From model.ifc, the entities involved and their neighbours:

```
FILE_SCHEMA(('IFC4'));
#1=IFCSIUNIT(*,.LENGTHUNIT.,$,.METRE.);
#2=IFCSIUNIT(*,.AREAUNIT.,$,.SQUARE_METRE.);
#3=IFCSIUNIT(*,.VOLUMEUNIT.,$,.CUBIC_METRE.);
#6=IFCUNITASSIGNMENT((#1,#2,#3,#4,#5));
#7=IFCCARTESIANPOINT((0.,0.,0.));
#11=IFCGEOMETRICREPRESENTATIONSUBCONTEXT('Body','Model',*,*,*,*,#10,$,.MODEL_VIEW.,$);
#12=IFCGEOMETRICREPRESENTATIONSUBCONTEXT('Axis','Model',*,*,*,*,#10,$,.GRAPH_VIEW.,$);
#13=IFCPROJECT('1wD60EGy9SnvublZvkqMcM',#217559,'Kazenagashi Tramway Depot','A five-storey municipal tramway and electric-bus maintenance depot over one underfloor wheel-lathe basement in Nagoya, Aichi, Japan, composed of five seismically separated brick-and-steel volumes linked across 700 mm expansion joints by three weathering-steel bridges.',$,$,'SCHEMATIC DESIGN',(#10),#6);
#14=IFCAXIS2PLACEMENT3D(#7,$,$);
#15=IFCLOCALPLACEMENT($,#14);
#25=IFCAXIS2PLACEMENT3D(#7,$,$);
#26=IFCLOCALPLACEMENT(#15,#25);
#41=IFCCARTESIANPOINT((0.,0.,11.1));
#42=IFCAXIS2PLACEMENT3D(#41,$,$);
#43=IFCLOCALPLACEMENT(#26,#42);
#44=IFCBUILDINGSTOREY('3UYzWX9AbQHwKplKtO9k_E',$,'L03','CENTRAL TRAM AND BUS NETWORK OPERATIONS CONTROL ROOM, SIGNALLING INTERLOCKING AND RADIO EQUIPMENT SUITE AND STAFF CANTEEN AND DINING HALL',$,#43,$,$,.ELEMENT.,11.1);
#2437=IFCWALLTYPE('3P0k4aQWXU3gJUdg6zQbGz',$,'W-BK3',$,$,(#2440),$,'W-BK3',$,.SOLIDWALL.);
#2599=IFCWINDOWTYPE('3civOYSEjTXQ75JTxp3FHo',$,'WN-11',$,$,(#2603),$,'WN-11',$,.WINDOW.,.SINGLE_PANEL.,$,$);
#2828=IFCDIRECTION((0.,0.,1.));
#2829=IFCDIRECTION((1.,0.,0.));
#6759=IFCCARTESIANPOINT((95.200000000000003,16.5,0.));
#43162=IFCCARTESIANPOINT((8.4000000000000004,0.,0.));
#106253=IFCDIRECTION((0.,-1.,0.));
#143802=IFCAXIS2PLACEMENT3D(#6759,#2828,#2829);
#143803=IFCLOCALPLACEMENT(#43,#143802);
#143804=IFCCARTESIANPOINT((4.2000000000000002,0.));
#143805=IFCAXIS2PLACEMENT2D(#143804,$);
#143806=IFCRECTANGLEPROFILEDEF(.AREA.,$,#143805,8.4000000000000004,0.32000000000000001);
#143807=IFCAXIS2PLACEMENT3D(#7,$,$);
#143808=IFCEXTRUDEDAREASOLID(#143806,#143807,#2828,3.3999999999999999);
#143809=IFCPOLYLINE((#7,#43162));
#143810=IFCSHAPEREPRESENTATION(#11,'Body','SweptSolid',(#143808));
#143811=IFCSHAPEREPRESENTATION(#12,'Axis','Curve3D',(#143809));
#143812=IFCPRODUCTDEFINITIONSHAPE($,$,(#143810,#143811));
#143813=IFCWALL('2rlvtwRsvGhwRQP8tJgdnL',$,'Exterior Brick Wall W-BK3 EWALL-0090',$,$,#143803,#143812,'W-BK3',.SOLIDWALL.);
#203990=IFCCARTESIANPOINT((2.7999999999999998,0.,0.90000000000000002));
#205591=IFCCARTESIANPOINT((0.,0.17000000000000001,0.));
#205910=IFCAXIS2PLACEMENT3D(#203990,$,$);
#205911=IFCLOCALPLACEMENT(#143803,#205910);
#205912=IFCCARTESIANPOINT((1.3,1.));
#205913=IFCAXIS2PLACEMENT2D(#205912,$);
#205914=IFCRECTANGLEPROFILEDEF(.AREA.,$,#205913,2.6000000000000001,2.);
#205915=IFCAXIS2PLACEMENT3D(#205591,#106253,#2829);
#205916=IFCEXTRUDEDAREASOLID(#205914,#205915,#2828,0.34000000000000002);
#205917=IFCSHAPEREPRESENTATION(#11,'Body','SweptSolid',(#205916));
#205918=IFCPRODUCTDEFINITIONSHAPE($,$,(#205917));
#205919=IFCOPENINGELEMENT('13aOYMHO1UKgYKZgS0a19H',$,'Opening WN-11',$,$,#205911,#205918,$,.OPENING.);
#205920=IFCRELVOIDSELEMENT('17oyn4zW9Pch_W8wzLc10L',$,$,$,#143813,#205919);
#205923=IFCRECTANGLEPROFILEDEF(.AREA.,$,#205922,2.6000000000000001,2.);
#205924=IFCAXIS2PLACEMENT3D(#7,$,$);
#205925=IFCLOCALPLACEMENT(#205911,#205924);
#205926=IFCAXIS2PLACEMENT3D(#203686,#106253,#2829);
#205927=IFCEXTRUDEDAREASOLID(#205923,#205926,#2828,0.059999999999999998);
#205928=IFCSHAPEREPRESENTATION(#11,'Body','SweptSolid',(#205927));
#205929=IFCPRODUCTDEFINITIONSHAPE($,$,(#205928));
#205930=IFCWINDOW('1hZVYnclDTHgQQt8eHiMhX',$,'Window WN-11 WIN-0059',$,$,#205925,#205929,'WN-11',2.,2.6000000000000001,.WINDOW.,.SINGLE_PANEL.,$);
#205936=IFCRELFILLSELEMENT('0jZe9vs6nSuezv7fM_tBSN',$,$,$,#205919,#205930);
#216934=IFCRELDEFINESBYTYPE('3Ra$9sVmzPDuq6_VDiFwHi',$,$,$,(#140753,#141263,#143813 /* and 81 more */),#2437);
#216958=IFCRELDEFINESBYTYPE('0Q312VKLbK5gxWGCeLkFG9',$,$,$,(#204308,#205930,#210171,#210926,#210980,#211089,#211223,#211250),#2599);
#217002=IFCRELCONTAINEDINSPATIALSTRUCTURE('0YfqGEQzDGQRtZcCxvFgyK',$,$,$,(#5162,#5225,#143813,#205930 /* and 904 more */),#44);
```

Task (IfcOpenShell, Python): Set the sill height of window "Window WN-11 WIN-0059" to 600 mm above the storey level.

```python
import numpy as np
import ifcopenshell
import ifcopenshell.api.geometry
import ifcopenshell.geom
import ifcopenshell.util.element
import ifcopenshell.util.placement
import ifcopenshell.util.shape
import ifcopenshell.util.unit

model = ifcopenshell.open("model.ifc")
unit_scale = ifcopenshell.util.unit.calculate_unit_scale(model)

window = model.by_id(205930)
opening = window.FillsVoids[0].RelatingOpeningElement
storey = ifcopenshell.util.element.get_container(window, ifc_class="IfcBuildingStorey")
level = ifcopenshell.util.placement.get_local_placement(storey.ObjectPlacement)[2, 3]

# The opening's origin need not be at the sill, so measure its lowest point.
shape = ifcopenshell.geom.create_shape(ifcopenshell.geom.settings(), opening)
bottom = ifcopenshell.util.shape.get_shape_bottom_elevation(shape, shape.geometry) / unit_scale
dz = level + 0.6 - bottom

shift = np.array([0.0, 0.0, dz])
# The window is placed relative to its opening, so it follows when the opening moves.
matrix = ifcopenshell.util.placement.get_local_placement(opening.ObjectPlacement)
matrix[:3, 3] += shift
ifcopenshell.api.geometry.edit_object_placement(
    model, product=opening, matrix=matrix, is_si=False, should_transform_children=True
)

print(f"moved by {dz * unit_scale:+.3f} m")

model.write("model_rev.ifc")
```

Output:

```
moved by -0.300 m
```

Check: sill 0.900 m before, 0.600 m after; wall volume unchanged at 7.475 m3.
